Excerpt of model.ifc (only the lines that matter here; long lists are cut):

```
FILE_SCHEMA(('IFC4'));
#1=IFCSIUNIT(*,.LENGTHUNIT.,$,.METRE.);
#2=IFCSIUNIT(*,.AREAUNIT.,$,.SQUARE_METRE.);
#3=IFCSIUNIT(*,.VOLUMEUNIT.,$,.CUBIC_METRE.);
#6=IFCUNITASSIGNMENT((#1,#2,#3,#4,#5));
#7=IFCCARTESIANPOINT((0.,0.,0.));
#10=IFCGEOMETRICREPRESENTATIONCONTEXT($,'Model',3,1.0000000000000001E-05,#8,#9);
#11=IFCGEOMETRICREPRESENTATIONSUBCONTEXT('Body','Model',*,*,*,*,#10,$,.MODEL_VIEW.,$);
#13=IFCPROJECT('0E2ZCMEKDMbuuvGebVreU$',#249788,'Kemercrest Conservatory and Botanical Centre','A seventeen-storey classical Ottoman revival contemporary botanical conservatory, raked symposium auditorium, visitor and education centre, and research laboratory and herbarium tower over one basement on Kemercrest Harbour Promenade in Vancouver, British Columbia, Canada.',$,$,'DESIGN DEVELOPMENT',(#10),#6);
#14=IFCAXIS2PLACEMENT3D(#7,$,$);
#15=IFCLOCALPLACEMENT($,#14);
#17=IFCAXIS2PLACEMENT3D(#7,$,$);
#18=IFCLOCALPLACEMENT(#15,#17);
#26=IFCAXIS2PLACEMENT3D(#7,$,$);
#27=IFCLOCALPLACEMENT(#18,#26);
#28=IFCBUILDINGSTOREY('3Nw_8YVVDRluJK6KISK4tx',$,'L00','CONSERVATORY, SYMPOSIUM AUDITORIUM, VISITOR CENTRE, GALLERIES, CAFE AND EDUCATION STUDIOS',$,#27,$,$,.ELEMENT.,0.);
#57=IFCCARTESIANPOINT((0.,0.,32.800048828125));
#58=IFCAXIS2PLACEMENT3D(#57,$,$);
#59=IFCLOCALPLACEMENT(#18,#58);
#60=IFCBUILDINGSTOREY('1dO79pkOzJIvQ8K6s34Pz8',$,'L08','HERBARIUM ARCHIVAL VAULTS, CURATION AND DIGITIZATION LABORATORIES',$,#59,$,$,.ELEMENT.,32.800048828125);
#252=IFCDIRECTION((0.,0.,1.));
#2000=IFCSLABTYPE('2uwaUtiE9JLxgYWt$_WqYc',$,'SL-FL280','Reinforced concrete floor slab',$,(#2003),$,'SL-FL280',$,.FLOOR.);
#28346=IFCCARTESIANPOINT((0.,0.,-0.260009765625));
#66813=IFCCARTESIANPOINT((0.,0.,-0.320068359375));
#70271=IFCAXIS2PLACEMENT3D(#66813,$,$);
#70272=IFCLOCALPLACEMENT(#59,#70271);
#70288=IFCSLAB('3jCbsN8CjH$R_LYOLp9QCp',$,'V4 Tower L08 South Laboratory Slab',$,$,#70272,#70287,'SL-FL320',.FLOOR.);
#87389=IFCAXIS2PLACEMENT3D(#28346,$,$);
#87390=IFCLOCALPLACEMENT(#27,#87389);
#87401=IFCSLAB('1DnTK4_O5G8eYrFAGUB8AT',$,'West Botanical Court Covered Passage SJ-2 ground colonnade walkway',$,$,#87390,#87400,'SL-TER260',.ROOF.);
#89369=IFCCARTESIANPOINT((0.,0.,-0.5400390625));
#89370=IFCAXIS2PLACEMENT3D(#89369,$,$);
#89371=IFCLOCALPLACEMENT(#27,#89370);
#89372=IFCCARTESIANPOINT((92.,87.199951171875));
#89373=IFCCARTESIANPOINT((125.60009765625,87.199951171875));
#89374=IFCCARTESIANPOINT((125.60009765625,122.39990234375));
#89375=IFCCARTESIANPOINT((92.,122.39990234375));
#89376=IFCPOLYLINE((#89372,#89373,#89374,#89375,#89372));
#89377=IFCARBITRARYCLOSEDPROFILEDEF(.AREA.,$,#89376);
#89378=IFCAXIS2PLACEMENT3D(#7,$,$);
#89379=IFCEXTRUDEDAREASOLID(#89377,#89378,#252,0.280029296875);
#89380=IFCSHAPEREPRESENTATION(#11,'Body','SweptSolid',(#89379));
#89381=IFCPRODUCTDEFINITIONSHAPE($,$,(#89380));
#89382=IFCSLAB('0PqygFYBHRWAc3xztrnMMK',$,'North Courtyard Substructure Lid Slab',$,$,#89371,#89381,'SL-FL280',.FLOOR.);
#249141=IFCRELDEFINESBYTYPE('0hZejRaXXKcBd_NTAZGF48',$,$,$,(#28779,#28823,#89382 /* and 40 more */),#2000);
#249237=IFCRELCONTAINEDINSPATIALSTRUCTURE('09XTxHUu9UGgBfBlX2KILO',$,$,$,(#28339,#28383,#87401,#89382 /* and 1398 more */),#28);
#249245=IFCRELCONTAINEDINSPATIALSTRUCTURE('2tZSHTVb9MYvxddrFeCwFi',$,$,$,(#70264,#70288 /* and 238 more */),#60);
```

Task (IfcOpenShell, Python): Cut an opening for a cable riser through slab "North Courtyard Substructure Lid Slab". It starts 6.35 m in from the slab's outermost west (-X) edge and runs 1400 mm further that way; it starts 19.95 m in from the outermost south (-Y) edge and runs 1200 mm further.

```python
import numpy as np
import ifcopenshell
import ifcopenshell.api.feature
import ifcopenshell.api.geometry
import ifcopenshell.api.root
import ifcopenshell.geom
import ifcopenshell.util.placement
import ifcopenshell.util.representation
import ifcopenshell.util.shape
import ifcopenshell.util.unit

model = ifcopenshell.open("model.ifc")
unit_scale = ifcopenshell.util.unit.calculate_unit_scale(model)
settings = ifcopenshell.geom.settings()


def volume(element):
    """Net volume in cubic metres, openings subtracted."""
    shape = ifcopenshell.geom.create_shape(settings, element)
    return ifcopenshell.util.shape.get_volume(shape.geometry)


slab = model.by_id(89382)
before = volume(slab)

# Extent in the slab's own axes, in metres. The edges named are its -X and -Y sides.
slab_shape = ifcopenshell.geom.create_shape(settings, slab)
vertices = ifcopenshell.util.shape.get_vertices(slab_shape.geometry)
x_min, y_min, bottom = vertices.min(axis=0)
top = vertices[:, 2].max()

opening = ifcopenshell.api.root.create_entity(model, ifc_class="IfcOpeningElement", name="Cable riser opening", predefined_type="OPENING")
context = ifcopenshell.util.representation.get_context(model, "Model", "Body", "MODEL_VIEW")
width, depth = 1.4, 1.2
outline = [(0.0, 0.0), (width, 0.0), (width, depth), (0.0, depth), (0.0, 0.0)]
# Overshoot both faces by 50 mm so the cut is clean.
shape = ifcopenshell.api.geometry.add_slab_representation(
    model, context=context, depth=top - bottom + 0.1, polyline=outline
)
ifcopenshell.api.geometry.assign_representation(model, product=opening, representation=shape)

matrix = ifcopenshell.util.placement.get_local_placement(slab.ObjectPlacement)
matrix[:, 3] = matrix @ np.append(np.array([x_min + 6.35, y_min + 19.95, bottom - 0.05]) / unit_scale, 1.0)
ifcopenshell.api.geometry.edit_object_placement(model, product=opening, matrix=matrix, is_si=False)
ifcopenshell.api.feature.add_feature(model, feature=opening, element=slab)

after = volume(slab)

print(f"slab volume {before:.3f} -> {after:.3f} m3")

model.write("model-out.ifc")
```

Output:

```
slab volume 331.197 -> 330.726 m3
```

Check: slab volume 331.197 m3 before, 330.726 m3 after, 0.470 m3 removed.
